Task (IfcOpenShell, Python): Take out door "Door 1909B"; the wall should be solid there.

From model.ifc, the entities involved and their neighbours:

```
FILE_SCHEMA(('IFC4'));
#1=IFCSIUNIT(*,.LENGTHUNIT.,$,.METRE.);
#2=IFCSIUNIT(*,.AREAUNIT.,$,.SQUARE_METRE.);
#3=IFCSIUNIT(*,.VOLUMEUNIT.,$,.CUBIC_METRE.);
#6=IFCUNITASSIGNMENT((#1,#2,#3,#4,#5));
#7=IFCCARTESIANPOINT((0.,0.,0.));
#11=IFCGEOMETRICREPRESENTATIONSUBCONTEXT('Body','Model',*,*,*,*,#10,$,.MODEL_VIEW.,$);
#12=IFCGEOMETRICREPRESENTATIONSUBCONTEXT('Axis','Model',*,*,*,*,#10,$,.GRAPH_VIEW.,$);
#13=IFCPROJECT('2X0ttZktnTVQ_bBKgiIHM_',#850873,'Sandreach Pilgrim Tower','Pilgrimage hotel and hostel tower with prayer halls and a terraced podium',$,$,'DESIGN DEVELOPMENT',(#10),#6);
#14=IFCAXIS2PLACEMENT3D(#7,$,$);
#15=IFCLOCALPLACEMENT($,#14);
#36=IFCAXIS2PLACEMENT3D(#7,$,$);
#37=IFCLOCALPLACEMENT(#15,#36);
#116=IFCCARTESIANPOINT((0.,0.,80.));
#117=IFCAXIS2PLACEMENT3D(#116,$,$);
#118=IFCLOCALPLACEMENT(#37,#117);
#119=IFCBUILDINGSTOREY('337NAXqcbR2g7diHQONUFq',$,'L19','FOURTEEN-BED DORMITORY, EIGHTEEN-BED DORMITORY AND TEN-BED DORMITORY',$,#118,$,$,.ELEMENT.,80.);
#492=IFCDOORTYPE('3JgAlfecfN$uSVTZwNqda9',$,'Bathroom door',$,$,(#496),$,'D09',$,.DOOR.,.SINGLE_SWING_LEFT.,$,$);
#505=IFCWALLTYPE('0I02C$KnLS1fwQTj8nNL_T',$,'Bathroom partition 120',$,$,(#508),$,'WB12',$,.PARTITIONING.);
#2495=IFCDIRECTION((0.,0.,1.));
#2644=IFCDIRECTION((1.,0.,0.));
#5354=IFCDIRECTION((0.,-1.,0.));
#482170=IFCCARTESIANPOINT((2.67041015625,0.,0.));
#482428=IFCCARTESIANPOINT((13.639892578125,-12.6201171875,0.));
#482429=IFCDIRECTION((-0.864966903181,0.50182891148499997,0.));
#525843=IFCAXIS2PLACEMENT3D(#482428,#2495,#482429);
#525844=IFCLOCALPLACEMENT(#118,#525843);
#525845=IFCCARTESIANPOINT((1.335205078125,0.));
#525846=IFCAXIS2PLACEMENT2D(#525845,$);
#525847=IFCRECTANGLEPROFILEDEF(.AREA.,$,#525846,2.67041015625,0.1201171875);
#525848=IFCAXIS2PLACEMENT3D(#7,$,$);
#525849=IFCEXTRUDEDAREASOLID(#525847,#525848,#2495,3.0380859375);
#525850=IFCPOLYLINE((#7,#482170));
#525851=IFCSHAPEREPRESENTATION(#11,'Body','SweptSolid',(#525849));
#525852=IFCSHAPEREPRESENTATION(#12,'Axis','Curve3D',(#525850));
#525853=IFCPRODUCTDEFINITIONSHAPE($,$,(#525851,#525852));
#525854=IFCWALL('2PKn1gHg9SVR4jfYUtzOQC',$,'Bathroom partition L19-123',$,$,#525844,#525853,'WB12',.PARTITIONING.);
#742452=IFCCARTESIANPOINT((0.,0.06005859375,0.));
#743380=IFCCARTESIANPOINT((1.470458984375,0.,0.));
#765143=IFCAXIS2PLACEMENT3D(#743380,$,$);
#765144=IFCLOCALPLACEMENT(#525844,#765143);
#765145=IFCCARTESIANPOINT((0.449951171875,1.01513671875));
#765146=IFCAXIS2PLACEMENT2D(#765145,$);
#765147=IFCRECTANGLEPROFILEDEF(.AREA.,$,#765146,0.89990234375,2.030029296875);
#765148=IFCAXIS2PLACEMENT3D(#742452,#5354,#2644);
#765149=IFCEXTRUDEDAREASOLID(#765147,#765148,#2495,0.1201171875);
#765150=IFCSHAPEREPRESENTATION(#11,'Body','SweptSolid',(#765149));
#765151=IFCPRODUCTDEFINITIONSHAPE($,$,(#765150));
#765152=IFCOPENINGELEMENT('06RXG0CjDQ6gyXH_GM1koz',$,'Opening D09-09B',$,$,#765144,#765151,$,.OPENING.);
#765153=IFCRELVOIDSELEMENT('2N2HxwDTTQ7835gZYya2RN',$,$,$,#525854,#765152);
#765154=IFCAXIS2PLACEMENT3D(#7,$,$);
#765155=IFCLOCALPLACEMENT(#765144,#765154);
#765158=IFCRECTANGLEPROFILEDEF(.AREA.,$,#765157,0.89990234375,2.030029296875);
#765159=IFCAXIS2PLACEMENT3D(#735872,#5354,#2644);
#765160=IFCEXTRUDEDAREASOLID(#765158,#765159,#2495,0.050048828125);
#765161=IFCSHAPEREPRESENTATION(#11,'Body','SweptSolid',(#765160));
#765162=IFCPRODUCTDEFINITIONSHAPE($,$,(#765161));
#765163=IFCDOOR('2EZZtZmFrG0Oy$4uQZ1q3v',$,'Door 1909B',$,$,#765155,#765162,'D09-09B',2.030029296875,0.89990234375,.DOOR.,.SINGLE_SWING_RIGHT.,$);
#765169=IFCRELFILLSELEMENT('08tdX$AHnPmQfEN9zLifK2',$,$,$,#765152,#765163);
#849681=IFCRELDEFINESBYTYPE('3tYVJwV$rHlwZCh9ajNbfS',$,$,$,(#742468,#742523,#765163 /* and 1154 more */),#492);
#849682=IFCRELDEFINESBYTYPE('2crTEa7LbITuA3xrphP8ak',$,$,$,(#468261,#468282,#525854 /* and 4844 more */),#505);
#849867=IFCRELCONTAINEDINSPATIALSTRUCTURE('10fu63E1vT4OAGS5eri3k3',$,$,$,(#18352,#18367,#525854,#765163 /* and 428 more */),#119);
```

```python
import ifcopenshell
import ifcopenshell.api.feature
import ifcopenshell.api.root
import ifcopenshell.geom
import ifcopenshell.util.shape

model = ifcopenshell.open("model.ifc")
settings = ifcopenshell.geom.settings()


def volume(element):
    """Net volume in cubic metres, openings subtracted."""
    shape = ifcopenshell.geom.create_shape(settings, element)
    return ifcopenshell.util.shape.get_volume(shape.geometry)


door = model.by_id(765163)
opening = door.FillsVoids[0].RelatingOpeningElement
wall = opening.VoidsElements[0].RelatingBuildingElement
before = volume(wall)

ifcopenshell.api.root.remove_product(model, product=door)
ifcopenshell.api.feature.remove_feature(model, feature=opening)

after = volume(wall)

print(f"wall volume {before:.3f} -> {after:.3f} m3")

model.write("model_v2.ifc")
```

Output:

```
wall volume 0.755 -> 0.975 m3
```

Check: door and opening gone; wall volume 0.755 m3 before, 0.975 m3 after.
